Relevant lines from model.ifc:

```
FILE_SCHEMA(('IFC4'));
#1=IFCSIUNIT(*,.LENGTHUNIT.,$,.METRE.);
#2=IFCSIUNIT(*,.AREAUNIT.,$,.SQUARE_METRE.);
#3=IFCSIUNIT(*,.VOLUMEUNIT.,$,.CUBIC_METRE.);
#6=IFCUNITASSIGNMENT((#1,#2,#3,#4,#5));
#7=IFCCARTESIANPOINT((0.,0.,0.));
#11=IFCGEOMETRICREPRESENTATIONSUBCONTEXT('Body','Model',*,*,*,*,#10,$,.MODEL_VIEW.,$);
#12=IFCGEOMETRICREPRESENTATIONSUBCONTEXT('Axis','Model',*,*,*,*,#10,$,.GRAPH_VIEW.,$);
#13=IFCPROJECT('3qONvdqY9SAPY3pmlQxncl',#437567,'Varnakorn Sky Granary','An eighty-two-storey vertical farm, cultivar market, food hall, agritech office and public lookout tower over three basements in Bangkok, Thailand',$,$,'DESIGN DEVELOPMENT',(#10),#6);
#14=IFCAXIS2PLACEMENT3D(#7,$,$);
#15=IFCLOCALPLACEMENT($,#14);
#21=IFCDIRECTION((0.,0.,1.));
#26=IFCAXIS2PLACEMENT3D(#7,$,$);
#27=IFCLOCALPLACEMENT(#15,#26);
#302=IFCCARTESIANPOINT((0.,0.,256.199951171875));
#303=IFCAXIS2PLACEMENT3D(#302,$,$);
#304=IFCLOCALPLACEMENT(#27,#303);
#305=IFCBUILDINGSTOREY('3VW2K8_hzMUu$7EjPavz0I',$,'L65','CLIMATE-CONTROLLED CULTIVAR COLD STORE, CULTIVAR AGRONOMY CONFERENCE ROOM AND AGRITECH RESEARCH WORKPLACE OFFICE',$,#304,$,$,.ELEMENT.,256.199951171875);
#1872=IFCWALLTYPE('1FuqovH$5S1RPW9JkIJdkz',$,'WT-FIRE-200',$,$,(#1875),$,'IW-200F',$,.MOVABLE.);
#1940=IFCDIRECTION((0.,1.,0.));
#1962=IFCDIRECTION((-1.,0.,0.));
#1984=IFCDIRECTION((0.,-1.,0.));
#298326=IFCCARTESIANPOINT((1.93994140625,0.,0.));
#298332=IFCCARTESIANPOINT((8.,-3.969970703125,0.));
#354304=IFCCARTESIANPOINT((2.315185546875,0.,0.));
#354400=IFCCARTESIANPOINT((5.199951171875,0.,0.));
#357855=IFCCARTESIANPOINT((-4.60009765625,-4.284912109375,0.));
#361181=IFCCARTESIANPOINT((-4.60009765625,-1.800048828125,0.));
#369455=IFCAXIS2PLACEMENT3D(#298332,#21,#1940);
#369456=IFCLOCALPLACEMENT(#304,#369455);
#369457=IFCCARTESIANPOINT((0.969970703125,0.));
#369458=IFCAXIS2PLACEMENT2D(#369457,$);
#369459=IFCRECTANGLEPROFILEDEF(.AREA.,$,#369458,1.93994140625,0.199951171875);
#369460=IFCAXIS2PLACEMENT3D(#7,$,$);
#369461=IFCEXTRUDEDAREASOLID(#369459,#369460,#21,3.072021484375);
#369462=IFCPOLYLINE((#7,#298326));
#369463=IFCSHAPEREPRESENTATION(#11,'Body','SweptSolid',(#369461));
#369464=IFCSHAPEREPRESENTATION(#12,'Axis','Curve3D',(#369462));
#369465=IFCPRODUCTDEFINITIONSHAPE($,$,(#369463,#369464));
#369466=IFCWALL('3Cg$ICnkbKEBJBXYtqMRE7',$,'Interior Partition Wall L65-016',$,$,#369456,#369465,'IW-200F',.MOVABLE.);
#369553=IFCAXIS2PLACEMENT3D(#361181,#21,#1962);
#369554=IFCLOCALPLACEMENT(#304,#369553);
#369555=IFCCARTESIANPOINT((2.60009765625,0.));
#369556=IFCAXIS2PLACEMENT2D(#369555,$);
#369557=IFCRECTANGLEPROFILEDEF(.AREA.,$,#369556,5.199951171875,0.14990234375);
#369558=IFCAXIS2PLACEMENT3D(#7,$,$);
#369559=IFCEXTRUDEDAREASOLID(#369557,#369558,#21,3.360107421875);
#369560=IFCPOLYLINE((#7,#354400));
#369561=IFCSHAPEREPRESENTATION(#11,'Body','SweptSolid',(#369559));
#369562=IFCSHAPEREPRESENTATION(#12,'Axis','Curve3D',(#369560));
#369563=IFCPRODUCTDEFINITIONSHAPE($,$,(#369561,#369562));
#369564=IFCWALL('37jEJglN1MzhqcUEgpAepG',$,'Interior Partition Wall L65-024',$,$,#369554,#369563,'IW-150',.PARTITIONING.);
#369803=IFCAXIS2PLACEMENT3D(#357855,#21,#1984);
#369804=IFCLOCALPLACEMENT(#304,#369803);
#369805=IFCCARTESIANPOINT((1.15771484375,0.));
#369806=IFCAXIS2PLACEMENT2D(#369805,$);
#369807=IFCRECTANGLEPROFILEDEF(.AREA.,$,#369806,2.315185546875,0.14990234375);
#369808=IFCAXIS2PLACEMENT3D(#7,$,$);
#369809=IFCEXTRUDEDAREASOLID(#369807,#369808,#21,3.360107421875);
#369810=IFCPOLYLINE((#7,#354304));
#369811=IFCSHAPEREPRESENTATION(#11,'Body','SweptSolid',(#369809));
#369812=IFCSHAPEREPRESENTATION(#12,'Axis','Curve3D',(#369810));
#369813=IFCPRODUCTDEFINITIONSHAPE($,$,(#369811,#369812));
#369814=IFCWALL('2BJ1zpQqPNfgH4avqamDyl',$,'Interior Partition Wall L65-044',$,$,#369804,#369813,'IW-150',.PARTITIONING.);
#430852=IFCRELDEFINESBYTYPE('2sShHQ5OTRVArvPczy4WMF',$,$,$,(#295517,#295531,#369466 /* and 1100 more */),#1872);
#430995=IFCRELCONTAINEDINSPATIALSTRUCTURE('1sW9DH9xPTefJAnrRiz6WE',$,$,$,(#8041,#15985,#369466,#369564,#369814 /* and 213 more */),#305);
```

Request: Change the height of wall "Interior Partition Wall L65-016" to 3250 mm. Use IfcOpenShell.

```python
import ifcopenshell
import ifcopenshell.geom
import ifcopenshell.util.representation
import ifcopenshell.util.shape
import ifcopenshell.util.unit

model = ifcopenshell.open("model.ifc")
unit_scale = ifcopenshell.util.unit.calculate_unit_scale(model)
settings = ifcopenshell.geom.settings()


def volume(element):
    """Net volume in cubic metres, openings subtracted."""
    shape = ifcopenshell.geom.create_shape(settings, element)
    return ifcopenshell.util.shape.get_volume(shape.geometry)


wall = model.by_guid("3Cg$ICnkbKEBJBXYtqMRE7")
before = volume(wall)

body = ifcopenshell.util.representation.get_representation(wall, "Model", "Body")
solid = body.Items[0]
old_height = solid.Depth
solid.Depth = 3.25 / unit_scale
after = volume(wall)

print(f"height {old_height:g} -> {solid.Depth:g}, volume {before:.3f} -> {after:.3f} m3")

model.write("model_rev.ifc")
```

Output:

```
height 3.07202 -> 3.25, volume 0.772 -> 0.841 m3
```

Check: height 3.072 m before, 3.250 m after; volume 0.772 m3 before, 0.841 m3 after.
